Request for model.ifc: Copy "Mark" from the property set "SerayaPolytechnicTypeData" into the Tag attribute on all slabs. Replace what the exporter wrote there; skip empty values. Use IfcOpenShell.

First a look at what the model holds.

```python
import ifcopenshell
import ifcopenshell.util.element

model = ifcopenshell.open("model.ifc")
print(model.schema)
slabs = model.by_type("IfcSlab")
print(len(slabs), "slabs")
for e in slabs[:8]:
    source = ifcopenshell.util.element.get_pset(e, "SerayaPolytechnicTypeData", "Mark")
    target = e.Tag
    print(e.id(), repr(source), repr(target), sep=" | ")
```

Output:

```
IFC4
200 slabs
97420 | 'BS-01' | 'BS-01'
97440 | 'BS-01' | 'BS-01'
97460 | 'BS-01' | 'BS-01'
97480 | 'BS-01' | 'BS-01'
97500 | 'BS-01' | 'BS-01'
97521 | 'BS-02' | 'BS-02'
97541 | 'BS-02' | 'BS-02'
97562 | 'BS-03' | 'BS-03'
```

```python
import ifcopenshell
import ifcopenshell.util.element

model = ifcopenshell.open("model.ifc")

count = 0
for e in model.by_type("IfcSlab"):
    value = ifcopenshell.util.element.get_pset(e, "SerayaPolytechnicTypeData", "Mark")
    current = e.Tag
    if not value or not value.strip() or current == value:
        continue
    e.Tag = value
    count += 1

print(count, "slabs updated")

model.write("model-out.ifc")
```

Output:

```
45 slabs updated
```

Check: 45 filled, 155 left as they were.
